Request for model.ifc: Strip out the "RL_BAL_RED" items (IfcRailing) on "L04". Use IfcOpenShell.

First a look at what the model holds.

```python
import ifcopenshell
import ifcopenshell.util.element

model = ifcopenshell.open("model.ifc")
print(model.schema)
storey = next(s for s in model.by_type("IfcBuildingStorey") if s.Name == "L04")
railings = [e for e in ifcopenshell.util.element.get_decomposition(storey) if e.is_a("IfcRailing")]
seen = {}
for e in railings:
    element_type = ifcopenshell.util.element.get_type(e)
    name = element_type.Name if element_type not in (None, e) else None
    seen[name] = seen.get(name, 0) + 1
for name, count in sorted(seen.items(), key=str):
    print(count, "x", name)
```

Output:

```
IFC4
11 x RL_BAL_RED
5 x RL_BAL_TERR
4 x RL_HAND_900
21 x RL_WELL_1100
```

```python
import ifcopenshell
import ifcopenshell.api.root
import ifcopenshell.util.element

model = ifcopenshell.open("model.ifc")

storey = next(s for s in model.by_type("IfcBuildingStorey") if s.Name == "L04")
railings = [e for e in ifcopenshell.util.element.get_decomposition(storey) if e.is_a("IfcRailing")]
targets = [e for e in railings if (t := ifcopenshell.util.element.get_type(e)) not in (None, e) and t.Name == "RL_BAL_RED"]

for e in targets:
    ifcopenshell.api.root.remove_product(model, product=e)
print(len(targets), "removed")

model.write("model-out.ifc")
```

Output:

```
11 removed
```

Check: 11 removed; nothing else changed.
